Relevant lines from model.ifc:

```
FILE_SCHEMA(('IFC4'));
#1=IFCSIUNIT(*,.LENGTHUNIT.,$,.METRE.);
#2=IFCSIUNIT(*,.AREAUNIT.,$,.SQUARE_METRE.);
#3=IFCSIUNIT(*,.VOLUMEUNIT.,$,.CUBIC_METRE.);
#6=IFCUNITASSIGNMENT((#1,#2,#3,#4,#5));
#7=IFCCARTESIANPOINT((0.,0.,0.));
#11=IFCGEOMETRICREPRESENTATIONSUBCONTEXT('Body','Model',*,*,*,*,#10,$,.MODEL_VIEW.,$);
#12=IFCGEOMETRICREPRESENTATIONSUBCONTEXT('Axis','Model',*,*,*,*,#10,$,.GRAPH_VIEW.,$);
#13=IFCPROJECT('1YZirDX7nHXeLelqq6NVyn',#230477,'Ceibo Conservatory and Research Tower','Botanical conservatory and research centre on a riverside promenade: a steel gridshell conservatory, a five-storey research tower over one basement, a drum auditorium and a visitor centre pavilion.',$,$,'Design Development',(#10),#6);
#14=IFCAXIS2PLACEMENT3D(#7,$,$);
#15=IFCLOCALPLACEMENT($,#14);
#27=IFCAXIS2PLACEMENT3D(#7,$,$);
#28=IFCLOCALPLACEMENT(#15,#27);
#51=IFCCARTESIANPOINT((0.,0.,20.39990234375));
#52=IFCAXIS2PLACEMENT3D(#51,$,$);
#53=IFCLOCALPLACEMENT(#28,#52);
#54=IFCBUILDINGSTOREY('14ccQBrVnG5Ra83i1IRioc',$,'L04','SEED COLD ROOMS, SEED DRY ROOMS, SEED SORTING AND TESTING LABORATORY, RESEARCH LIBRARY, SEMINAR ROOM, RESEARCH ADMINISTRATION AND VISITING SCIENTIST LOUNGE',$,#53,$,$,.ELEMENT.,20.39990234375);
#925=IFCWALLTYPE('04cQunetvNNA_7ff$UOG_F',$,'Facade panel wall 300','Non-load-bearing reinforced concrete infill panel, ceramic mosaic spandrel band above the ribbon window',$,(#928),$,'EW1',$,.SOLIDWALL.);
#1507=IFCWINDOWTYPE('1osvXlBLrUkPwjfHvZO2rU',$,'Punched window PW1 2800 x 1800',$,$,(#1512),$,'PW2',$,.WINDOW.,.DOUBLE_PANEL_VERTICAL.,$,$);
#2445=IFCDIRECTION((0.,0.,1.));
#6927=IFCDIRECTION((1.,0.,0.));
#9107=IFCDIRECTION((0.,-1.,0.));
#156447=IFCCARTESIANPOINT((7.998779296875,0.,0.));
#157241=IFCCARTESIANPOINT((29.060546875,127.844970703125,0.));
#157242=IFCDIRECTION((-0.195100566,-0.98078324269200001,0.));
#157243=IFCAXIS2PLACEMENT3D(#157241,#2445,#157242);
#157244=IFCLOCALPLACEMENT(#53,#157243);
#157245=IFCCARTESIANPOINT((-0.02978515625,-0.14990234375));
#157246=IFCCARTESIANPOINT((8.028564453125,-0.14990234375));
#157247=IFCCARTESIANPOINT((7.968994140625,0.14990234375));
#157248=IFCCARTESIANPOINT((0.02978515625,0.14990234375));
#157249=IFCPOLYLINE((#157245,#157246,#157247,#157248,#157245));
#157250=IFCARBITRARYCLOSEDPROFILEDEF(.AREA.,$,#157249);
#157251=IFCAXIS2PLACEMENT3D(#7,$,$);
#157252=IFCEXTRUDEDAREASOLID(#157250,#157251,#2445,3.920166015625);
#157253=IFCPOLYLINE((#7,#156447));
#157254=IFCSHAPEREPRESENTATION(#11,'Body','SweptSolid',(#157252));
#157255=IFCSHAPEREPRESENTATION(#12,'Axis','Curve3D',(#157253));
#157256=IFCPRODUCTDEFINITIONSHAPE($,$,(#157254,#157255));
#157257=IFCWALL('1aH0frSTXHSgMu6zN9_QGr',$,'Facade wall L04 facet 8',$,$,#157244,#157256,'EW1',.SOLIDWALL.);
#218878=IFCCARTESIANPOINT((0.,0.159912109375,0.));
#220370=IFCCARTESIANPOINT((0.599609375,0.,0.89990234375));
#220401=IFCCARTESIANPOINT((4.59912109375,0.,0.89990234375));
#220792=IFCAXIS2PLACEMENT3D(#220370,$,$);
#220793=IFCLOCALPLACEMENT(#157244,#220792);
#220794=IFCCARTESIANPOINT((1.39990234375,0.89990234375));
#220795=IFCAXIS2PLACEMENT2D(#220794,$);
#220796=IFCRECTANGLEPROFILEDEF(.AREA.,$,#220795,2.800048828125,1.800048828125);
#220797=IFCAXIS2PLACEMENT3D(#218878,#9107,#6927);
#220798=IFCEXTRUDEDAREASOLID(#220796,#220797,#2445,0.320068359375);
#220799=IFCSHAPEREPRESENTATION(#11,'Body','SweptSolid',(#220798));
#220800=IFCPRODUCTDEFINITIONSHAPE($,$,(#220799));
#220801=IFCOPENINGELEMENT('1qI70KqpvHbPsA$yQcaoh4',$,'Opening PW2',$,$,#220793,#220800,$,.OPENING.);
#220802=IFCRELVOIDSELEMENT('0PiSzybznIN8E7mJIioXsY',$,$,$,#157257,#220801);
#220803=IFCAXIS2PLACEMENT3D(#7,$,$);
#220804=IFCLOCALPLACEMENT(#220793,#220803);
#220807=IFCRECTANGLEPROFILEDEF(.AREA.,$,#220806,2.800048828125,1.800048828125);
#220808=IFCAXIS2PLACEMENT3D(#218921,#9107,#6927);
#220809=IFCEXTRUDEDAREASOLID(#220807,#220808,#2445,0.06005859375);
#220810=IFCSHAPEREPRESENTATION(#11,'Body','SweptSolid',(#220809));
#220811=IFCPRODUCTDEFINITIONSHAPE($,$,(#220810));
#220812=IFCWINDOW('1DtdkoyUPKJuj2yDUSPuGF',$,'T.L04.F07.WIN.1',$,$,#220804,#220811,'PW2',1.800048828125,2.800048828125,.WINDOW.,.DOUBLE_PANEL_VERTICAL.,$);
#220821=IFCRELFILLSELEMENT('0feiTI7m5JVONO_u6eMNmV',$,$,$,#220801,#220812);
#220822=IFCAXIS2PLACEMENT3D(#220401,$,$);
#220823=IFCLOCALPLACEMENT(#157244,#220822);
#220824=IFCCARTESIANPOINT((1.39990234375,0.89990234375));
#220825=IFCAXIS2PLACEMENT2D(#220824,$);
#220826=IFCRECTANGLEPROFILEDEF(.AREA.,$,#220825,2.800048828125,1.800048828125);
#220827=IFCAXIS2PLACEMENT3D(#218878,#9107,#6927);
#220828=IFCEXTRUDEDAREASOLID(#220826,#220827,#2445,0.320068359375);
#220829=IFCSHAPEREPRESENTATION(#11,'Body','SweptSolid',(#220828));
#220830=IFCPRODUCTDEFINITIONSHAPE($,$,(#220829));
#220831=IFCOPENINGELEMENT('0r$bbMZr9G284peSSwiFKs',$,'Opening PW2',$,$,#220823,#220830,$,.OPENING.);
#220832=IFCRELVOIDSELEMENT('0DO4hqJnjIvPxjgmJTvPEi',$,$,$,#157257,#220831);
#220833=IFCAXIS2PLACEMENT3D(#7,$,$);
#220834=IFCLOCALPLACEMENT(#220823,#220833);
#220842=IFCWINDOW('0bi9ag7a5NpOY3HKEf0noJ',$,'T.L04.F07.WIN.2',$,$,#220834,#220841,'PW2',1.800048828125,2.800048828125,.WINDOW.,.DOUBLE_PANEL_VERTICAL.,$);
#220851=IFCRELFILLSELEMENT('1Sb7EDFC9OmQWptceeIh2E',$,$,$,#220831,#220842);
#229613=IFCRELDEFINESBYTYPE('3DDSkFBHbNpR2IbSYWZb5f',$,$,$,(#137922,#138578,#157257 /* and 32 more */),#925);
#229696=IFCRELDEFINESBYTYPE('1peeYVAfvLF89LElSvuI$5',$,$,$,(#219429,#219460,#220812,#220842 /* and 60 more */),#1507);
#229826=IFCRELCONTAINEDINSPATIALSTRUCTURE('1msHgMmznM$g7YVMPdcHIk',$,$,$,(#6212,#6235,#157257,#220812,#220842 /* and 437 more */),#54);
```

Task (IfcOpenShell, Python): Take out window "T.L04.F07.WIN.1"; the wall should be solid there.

```python
import ifcopenshell
import ifcopenshell.api.feature
import ifcopenshell.api.root
import ifcopenshell.geom
import ifcopenshell.util.shape

model = ifcopenshell.open("model.ifc")
settings = ifcopenshell.geom.settings()


def volume(element):
    """Net volume in cubic metres, openings subtracted."""
    shape = ifcopenshell.geom.create_shape(settings, element)
    return ifcopenshell.util.shape.get_volume(shape.geometry)


window = model.by_guid("1DtdkoyUPKJuj2yDUSPuGF")
opening = window.FillsVoids[0].RelatingOpeningElement
wall = opening.VoidsElements[0].RelatingBuildingElement
before = volume(wall)

ifcopenshell.api.root.remove_product(model, product=window)
ifcopenshell.api.feature.remove_feature(model, feature=opening)

after = volume(wall)

print(f"wall volume {before:.3f} -> {after:.3f} m3")

model.write("model_edited.ifc")
```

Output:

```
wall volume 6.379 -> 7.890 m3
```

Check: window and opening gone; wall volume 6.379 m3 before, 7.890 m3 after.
